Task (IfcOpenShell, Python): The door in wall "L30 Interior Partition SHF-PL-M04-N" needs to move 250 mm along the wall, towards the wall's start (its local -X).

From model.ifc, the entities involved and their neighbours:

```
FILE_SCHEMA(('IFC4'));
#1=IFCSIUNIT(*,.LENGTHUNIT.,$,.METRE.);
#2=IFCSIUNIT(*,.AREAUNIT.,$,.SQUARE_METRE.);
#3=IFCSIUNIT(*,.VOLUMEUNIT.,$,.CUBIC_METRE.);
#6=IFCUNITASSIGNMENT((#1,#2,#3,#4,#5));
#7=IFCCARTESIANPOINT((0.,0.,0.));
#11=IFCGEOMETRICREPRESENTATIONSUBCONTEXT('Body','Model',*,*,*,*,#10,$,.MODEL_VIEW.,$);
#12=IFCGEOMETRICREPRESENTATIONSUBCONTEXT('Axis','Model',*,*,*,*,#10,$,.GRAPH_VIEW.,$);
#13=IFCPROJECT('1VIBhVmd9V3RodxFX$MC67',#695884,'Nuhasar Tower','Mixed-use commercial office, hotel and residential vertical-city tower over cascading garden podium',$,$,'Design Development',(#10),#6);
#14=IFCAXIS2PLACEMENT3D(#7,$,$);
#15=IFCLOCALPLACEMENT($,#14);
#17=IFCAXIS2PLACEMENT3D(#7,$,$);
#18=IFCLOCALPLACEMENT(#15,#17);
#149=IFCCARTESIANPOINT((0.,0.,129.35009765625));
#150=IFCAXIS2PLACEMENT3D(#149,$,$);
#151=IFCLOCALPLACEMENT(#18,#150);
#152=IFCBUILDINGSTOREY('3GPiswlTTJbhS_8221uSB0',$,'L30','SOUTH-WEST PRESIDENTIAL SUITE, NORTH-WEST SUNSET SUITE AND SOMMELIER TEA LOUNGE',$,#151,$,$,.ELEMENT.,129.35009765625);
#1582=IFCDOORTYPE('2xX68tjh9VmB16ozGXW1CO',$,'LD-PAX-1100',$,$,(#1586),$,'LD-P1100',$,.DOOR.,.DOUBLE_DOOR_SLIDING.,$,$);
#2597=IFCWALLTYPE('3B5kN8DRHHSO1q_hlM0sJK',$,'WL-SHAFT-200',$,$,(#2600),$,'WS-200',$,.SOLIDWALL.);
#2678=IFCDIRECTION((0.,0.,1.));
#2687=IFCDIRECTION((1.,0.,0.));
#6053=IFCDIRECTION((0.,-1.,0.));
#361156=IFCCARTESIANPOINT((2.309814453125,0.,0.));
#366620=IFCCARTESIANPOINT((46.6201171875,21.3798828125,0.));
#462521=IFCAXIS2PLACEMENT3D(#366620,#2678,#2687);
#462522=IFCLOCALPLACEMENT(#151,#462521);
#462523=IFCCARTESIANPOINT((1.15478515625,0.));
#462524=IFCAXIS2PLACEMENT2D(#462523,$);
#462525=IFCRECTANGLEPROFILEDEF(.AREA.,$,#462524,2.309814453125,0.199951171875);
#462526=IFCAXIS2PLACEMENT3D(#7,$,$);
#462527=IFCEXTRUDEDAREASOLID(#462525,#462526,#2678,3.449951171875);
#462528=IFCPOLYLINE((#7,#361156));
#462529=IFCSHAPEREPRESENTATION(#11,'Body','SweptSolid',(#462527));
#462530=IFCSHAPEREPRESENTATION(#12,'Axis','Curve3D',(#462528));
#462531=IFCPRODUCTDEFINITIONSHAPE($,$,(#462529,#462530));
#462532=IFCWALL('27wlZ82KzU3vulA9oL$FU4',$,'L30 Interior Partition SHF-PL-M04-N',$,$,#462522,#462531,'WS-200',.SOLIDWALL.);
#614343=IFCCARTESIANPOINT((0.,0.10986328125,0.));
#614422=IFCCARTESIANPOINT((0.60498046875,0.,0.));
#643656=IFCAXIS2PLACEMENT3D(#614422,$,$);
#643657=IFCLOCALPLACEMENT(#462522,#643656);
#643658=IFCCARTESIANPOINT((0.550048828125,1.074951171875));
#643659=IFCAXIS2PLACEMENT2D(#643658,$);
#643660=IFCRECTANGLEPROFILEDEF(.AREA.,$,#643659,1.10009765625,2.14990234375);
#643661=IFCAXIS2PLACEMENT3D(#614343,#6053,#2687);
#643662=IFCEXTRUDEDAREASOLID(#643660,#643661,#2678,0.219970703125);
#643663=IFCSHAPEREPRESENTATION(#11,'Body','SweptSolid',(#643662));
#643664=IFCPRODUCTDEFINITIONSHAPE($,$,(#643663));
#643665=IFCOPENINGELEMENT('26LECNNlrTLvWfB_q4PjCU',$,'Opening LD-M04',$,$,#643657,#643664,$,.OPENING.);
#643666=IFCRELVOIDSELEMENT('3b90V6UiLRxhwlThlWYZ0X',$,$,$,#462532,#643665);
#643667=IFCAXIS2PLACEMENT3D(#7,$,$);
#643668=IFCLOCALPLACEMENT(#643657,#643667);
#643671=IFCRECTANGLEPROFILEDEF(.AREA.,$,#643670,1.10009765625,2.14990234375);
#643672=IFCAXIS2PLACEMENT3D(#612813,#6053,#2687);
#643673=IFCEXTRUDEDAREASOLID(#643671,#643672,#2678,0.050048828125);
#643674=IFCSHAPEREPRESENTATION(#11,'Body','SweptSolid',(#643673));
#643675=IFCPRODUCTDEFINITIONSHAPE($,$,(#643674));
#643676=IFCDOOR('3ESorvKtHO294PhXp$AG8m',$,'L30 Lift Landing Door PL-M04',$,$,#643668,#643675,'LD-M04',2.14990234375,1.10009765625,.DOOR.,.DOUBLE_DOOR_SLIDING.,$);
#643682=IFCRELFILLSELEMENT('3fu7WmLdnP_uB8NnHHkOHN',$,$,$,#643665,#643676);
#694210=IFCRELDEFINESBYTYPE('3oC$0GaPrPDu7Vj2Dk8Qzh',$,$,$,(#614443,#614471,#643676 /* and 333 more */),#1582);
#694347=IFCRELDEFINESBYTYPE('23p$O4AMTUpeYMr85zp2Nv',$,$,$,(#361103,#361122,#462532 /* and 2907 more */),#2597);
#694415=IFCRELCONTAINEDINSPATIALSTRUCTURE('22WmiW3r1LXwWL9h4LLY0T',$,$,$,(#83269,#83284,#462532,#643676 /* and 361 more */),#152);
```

```python
import ifcopenshell
import ifcopenshell.api.geometry
import ifcopenshell.util.placement

model = ifcopenshell.open("model.ifc")

door = model.by_guid("3ESorvKtHO294PhXp$AG8m")
opening = door.FillsVoids[0].RelatingOpeningElement
wall = opening.VoidsElements[0].RelatingBuildingElement

wall_matrix = ifcopenshell.util.placement.get_local_placement(wall.ObjectPlacement)
shift = wall_matrix[:3, 0] * -0.25
before = ifcopenshell.util.placement.get_local_placement(door.ObjectPlacement)[:3, 3].copy()

# The door is placed relative to its opening, so it follows when the opening moves.
matrix = ifcopenshell.util.placement.get_local_placement(opening.ObjectPlacement)
matrix[:3, 3] += shift
ifcopenshell.api.geometry.edit_object_placement(
    model, product=opening, matrix=matrix, is_si=False, should_transform_children=True
)

after = ifcopenshell.util.placement.get_local_placement(door.ObjectPlacement)[:3, 3]
print("door moved by", (after - before).round(3) + 0.0)

model.write("model_rev.ifc")
```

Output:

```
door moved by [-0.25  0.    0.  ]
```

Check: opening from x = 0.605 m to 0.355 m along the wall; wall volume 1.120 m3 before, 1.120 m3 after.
